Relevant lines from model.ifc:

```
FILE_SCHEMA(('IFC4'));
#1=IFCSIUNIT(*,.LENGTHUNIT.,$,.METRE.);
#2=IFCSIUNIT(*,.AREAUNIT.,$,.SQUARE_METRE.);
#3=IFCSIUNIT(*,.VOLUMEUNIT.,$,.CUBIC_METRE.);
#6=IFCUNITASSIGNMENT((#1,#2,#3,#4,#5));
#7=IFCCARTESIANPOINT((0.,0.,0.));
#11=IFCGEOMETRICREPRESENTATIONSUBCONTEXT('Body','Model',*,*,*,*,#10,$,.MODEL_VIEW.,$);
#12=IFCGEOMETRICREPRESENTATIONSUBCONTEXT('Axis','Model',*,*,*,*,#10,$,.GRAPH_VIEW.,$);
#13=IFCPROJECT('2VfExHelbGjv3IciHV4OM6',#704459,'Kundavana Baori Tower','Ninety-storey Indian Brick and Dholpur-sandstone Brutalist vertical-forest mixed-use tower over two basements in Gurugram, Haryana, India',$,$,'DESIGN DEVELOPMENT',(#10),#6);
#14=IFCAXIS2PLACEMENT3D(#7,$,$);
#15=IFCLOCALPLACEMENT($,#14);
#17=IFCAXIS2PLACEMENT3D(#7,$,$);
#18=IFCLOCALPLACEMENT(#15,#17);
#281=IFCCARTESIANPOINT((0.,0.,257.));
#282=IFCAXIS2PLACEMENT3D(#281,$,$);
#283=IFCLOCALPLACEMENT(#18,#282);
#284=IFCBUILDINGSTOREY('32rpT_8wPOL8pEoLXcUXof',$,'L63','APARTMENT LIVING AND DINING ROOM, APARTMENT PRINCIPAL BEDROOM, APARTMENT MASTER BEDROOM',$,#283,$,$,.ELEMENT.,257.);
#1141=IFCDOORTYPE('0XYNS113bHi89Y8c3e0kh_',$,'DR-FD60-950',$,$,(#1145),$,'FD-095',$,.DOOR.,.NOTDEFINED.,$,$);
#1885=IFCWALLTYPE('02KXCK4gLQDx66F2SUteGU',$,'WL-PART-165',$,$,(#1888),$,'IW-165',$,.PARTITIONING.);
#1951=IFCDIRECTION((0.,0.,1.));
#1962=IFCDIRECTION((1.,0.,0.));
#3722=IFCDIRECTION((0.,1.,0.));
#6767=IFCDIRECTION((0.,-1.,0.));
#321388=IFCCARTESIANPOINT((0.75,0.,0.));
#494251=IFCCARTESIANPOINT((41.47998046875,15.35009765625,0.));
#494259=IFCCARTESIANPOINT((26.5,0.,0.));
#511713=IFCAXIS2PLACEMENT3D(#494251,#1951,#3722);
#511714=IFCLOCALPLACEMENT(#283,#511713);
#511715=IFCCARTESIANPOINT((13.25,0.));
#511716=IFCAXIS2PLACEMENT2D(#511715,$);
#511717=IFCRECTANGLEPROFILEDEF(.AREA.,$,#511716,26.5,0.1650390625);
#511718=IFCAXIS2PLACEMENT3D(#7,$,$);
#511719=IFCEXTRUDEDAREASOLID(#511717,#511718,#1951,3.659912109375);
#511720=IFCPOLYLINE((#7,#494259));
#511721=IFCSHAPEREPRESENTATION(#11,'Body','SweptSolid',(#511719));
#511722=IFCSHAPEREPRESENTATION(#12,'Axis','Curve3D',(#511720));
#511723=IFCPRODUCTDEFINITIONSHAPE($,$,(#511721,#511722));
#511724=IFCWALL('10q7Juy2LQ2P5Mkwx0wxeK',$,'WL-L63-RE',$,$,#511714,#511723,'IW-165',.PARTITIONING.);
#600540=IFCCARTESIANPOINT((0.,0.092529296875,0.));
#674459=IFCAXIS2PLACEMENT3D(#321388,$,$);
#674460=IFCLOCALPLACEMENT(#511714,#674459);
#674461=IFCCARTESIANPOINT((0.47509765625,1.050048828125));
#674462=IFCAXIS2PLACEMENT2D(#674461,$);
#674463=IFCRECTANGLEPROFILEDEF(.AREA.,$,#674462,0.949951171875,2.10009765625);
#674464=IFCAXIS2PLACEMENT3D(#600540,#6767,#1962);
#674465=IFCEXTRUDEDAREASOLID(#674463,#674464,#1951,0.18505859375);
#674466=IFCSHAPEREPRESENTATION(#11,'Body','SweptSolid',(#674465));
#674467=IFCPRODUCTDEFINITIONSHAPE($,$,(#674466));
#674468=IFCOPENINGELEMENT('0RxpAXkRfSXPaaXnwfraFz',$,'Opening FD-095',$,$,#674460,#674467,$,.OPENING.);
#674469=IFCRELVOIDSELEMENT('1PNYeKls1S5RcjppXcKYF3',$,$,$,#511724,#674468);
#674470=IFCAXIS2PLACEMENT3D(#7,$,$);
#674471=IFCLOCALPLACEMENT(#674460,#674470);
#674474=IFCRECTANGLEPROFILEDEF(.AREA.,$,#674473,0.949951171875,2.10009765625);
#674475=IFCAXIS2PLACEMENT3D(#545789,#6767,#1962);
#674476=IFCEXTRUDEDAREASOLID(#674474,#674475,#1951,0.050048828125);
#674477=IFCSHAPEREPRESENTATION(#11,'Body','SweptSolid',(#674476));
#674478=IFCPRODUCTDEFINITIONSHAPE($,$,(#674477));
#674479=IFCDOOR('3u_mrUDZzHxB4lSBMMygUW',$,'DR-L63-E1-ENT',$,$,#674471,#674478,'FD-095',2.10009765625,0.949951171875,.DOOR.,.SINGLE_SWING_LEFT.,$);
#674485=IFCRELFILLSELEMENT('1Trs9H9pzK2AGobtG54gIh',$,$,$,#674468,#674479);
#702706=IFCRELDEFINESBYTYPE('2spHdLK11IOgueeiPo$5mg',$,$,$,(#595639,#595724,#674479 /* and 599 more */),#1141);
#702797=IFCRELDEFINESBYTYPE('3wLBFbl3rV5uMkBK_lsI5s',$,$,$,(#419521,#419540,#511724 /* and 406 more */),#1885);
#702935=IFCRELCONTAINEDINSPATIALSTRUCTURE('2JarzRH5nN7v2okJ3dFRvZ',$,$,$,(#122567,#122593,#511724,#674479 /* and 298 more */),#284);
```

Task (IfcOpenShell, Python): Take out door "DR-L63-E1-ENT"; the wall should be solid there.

```python
import ifcopenshell
import ifcopenshell.api.feature
import ifcopenshell.api.root
import ifcopenshell.geom
import ifcopenshell.util.shape

model = ifcopenshell.open("model.ifc")
settings = ifcopenshell.geom.settings()


def volume(element):
    """Net volume in cubic metres, openings subtracted."""
    shape = ifcopenshell.geom.create_shape(settings, element)
    return ifcopenshell.util.shape.get_volume(shape.geometry)


door = model.by_id(674479)
opening = door.FillsVoids[0].RelatingOpeningElement
wall = opening.VoidsElements[0].RelatingBuildingElement
before = volume(wall)

ifcopenshell.api.root.remove_product(model, product=door)
ifcopenshell.api.feature.remove_feature(model, feature=opening)

after = volume(wall)

print(f"wall volume {before:.3f} -> {after:.3f} m3")

model.write("model_updated.ifc")
```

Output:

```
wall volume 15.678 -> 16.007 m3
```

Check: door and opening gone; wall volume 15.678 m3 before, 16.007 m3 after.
